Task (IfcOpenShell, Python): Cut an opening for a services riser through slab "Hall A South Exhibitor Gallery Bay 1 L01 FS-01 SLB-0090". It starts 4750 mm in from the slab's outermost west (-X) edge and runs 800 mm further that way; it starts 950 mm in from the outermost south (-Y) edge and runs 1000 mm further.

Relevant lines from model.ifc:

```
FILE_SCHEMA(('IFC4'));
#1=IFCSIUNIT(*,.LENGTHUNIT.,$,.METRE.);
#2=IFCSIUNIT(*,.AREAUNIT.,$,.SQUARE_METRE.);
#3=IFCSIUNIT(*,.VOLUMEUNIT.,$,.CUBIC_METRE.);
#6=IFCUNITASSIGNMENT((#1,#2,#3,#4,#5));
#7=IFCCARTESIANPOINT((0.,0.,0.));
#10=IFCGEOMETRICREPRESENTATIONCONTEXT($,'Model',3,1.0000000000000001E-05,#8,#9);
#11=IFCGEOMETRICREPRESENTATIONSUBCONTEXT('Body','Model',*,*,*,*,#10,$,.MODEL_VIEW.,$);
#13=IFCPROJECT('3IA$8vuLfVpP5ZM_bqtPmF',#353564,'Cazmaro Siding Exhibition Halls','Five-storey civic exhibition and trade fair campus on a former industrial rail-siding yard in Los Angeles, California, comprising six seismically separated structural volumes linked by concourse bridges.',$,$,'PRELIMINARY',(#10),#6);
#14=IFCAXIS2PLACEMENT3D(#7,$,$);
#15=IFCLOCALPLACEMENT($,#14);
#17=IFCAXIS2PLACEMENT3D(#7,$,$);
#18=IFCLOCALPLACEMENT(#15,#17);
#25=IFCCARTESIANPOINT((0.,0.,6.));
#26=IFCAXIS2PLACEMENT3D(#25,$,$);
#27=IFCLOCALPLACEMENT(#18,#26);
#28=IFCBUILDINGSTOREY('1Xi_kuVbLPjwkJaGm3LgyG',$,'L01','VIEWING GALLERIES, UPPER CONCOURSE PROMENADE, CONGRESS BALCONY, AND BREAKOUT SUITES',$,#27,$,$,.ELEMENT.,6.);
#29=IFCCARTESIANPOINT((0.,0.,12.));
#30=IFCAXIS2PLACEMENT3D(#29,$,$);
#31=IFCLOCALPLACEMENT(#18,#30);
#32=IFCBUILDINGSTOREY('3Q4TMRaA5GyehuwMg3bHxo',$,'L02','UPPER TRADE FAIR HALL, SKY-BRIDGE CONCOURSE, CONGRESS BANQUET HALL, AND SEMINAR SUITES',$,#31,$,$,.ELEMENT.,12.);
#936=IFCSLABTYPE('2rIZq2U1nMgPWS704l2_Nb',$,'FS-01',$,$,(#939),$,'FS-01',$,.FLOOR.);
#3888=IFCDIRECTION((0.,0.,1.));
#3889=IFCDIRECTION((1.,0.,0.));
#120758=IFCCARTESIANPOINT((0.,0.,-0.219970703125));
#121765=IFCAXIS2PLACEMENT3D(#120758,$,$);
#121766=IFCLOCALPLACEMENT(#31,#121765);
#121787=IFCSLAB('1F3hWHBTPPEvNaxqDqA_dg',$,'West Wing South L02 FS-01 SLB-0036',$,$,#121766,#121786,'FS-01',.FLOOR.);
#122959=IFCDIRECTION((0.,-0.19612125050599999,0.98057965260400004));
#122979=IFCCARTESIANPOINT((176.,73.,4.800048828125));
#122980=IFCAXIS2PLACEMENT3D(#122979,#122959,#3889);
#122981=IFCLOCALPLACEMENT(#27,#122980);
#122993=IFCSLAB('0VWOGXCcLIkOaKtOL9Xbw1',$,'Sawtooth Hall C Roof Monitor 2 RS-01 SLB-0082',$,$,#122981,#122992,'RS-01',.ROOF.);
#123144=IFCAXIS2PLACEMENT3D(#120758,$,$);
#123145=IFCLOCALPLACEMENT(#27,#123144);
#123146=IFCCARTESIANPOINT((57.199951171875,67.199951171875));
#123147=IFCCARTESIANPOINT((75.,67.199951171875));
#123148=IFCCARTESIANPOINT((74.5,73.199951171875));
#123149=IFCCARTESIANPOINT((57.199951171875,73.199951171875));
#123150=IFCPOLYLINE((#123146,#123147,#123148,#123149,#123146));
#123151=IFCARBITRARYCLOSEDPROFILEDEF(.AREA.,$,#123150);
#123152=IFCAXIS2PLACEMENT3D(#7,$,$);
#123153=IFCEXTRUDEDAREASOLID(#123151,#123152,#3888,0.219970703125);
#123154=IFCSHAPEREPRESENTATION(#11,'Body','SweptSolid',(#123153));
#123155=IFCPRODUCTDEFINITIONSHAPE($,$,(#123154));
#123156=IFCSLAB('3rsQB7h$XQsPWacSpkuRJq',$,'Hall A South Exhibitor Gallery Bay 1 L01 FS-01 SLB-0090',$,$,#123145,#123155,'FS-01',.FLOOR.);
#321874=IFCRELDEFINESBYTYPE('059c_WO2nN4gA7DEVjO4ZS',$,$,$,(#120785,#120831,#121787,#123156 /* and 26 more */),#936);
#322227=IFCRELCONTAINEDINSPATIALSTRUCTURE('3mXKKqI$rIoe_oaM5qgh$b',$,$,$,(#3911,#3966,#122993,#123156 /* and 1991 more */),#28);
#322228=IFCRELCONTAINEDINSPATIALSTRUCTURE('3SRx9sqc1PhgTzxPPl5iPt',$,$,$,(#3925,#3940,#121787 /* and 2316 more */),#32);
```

```python
import numpy as np
import ifcopenshell
import ifcopenshell.api.feature
import ifcopenshell.api.geometry
import ifcopenshell.api.root
import ifcopenshell.geom
import ifcopenshell.util.placement
import ifcopenshell.util.representation
import ifcopenshell.util.shape
import ifcopenshell.util.unit

model = ifcopenshell.open("model.ifc")
unit_scale = ifcopenshell.util.unit.calculate_unit_scale(model)
settings = ifcopenshell.geom.settings()


def volume(element):
    """Net volume in cubic metres, openings subtracted."""
    shape = ifcopenshell.geom.create_shape(settings, element)
    return ifcopenshell.util.shape.get_volume(shape.geometry)


slab = model.by_guid("3rsQB7h$XQsPWacSpkuRJq")
before = volume(slab)

# Extent in the slab's own axes, in metres. The edges named are its -X and -Y sides.
slab_shape = ifcopenshell.geom.create_shape(settings, slab)
vertices = ifcopenshell.util.shape.get_vertices(slab_shape.geometry)
x_min, y_min, bottom = vertices.min(axis=0)
top = vertices[:, 2].max()

opening = ifcopenshell.api.root.create_entity(model, ifc_class="IfcOpeningElement", name="Services riser opening", predefined_type="OPENING")
context = ifcopenshell.util.representation.get_context(model, "Model", "Body", "MODEL_VIEW")
width, depth = 0.8, 1
outline = [(0.0, 0.0), (width, 0.0), (width, depth), (0.0, depth), (0.0, 0.0)]
# Overshoot both faces by 50 mm so the cut is clean.
shape = ifcopenshell.api.geometry.add_slab_representation(
    model, context=context, depth=top - bottom + 0.1, polyline=outline
)
ifcopenshell.api.geometry.assign_representation(model, product=opening, representation=shape)

matrix = ifcopenshell.util.placement.get_local_placement(slab.ObjectPlacement)
matrix[:, 3] = matrix @ np.append(np.array([x_min + 4.75, y_min + 0.95, bottom - 0.05]) / unit_scale, 1.0)
ifcopenshell.api.geometry.edit_object_placement(model, product=opening, matrix=matrix, is_si=False)
ifcopenshell.api.feature.add_feature(model, feature=opening, element=slab)

after = volume(slab)

print(f"slab volume {before:.3f} -> {after:.3f} m3")

model.write("model_updated.ifc")
```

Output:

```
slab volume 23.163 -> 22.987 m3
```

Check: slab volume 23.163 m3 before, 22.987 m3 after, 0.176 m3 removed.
